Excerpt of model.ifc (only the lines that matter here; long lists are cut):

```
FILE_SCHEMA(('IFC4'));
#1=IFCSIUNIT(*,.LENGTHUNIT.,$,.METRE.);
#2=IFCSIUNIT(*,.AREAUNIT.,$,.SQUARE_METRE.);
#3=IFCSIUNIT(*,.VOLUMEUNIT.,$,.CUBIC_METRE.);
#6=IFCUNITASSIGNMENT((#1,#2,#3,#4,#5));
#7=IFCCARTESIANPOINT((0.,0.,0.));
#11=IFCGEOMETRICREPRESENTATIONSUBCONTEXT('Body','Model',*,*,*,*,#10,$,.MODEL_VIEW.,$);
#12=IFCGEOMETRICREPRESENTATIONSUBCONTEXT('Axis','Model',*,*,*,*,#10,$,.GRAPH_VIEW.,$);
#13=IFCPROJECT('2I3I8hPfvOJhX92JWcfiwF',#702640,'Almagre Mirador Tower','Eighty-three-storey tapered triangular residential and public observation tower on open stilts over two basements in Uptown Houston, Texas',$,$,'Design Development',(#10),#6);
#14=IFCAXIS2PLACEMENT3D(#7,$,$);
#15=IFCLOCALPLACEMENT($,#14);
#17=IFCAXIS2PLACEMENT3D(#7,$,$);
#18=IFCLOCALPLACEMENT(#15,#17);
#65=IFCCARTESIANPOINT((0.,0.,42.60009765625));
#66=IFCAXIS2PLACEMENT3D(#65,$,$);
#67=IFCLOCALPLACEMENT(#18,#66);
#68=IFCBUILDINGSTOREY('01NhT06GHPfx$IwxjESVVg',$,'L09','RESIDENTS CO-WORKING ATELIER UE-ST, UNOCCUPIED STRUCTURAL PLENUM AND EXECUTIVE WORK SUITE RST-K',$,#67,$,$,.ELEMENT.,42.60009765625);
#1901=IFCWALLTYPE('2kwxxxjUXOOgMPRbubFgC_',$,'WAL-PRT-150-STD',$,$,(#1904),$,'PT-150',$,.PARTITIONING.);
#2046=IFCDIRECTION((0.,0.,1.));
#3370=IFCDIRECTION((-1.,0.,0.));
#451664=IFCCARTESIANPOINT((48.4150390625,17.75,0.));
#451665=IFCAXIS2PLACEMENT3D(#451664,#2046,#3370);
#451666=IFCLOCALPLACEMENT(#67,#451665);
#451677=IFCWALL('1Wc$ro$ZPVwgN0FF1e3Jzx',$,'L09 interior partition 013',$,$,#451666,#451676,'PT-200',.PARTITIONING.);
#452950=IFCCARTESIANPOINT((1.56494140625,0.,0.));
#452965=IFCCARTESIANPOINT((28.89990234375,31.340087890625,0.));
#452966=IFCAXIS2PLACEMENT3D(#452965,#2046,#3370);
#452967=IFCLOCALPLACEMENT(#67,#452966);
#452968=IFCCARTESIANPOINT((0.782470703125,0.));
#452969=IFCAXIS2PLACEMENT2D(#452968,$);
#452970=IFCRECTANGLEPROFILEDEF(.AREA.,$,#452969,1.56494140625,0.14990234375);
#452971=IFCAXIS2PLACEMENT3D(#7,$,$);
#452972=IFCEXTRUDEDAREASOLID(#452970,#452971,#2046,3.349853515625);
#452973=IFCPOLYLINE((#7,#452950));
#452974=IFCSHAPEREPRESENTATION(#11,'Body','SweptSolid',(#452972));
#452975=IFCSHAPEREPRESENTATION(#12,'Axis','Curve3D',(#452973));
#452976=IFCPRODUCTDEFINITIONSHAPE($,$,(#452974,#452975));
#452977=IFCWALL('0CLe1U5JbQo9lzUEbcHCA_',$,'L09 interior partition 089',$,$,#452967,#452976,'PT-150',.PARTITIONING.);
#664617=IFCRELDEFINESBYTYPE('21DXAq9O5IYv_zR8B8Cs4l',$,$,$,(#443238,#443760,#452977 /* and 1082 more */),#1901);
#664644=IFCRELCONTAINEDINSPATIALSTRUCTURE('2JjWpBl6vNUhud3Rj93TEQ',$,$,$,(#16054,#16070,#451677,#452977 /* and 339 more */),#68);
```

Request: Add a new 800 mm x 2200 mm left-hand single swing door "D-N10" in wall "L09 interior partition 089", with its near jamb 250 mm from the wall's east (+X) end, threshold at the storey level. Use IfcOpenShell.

```python
import numpy as np
import ifcopenshell
import ifcopenshell.api.feature
import ifcopenshell.api.geometry
import ifcopenshell.api.root
import ifcopenshell.api.spatial
import ifcopenshell.geom
import ifcopenshell.util.element
import ifcopenshell.util.placement
import ifcopenshell.util.representation
import ifcopenshell.util.shape
import ifcopenshell.util.unit

model = ifcopenshell.open("model.ifc")
unit_scale = ifcopenshell.util.unit.calculate_unit_scale(model)
settings = ifcopenshell.geom.settings()


def volume(element):
    """Net volume in cubic metres, openings subtracted."""
    shape = ifcopenshell.geom.create_shape(settings, element)
    return ifcopenshell.util.shape.get_volume(shape.geometry)


wall = model.by_id(452977)
storey = ifcopenshell.util.element.get_container(wall, ifc_class="IfcBuildingStorey")
context = ifcopenshell.util.representation.get_context(model, "Model", "Body", "MODEL_VIEW")
before = volume(wall)

width, height, from_end, sill = 0.8, 2.2, 0.25, 0.0  # metres

# The wall runs along its own X axis, and the end named is its -X end.
wall_shape = ifcopenshell.geom.create_shape(settings, wall)
x, y, z = ifcopenshell.util.shape.get_vertices(wall_shape.geometry).T
start = x.min() + from_end
face, thickness = float(y.min()), float(y.max() - y.min())
wall_matrix = ifcopenshell.util.placement.get_local_placement(wall.ObjectPlacement)
level = ifcopenshell.util.placement.get_local_placement(storey.ObjectPlacement)[2, 3]


def in_wall(x, y):
    """Placement at x, y metres in the wall's axes, at sill height."""
    matrix = wall_matrix.copy()
    matrix[:, 3] = wall_matrix @ np.array([x / unit_scale, y / unit_scale, 0.0, 1.0])
    matrix[2, 3] = level + sill / unit_scale
    return matrix


# Opening: a box that overshoots both wall faces by 50 mm.
opening = ifcopenshell.api.root.create_entity(model, ifc_class="IfcOpeningElement", predefined_type="OPENING")
box = ifcopenshell.api.geometry.add_wall_representation(
    model, context=context, length=width, height=height, thickness=thickness + 0.1
)
ifcopenshell.api.geometry.assign_representation(model, product=opening, representation=box)
ifcopenshell.api.geometry.edit_object_placement(model, product=opening, matrix=in_wall(start, face - 0.05), is_si=False)
ifcopenshell.api.feature.add_feature(model, feature=opening, element=wall)

door = ifcopenshell.api.root.create_entity(model, ifc_class="IfcDoor", name="D-N10", predefined_type="DOOR")
door.OverallWidth, door.OverallHeight = width / unit_scale, height / unit_scale
door.OperationType = "SINGLE_SWING_LEFT"
body = ifcopenshell.api.geometry.add_door_representation(
    model,
    context=context,
    overall_width=door.OverallWidth,
    overall_height=door.OverallHeight,
    operation_type="SINGLE_SWING_LEFT",
    lining_properties={"LiningDepth": thickness / unit_scale, "ThresholdDepth": thickness / unit_scale},
)
ifcopenshell.api.geometry.assign_representation(model, product=door, representation=body)
ifcopenshell.api.spatial.assign_container(model, products=[door], relating_structure=storey)
ifcopenshell.api.feature.add_filling(model, opening=opening, element=door)

# The lining spans the wall, so the door starts at the wall face.
ifcopenshell.api.geometry.edit_object_placement(model, product=door, matrix=in_wall(start, face), is_si=False)

after = volume(wall)

print(f"wall volume {before:.3f} -> {after:.3f} m3")

model.write("model_v2.ifc")
```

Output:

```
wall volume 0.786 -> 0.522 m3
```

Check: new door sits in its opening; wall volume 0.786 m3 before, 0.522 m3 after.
